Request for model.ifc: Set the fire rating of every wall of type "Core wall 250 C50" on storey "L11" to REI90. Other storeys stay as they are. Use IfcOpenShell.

First a look at what the model holds.

```python
import ifcopenshell
import ifcopenshell.util.element

model = ifcopenshell.open("model.ifc")
print(model.schema)
storey = next(s for s in model.by_type("IfcBuildingStorey") if s.Name == "L11")
walls = [e for e in ifcopenshell.util.element.get_decomposition(storey) if e.is_a("IfcWall")]
seen = {}
for e in walls:
    element_type = ifcopenshell.util.element.get_type(e)
    key = (element_type.Name if element_type != e and element_type else None, ifcopenshell.util.element.get_pset(e, "Pset_WallCommon", "FireRating"))
    seen[key] = seen.get(key, 0) + 1
for (name, value), count in sorted(seen.items(), key=str):
    print(count, "x", name, "|", value)
```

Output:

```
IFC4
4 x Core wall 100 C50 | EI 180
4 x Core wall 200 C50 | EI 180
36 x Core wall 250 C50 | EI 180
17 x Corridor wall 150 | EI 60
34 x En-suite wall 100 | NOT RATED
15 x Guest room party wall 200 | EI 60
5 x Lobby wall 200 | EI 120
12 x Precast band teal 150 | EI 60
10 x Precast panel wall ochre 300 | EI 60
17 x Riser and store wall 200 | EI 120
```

```python
import ifcopenshell
import ifcopenshell.api.pset
import ifcopenshell.util.element

model = ifcopenshell.open("model.ifc")

storey = next(s for s in model.by_type("IfcBuildingStorey") if s.Name == "L11")
walls = [e for e in ifcopenshell.util.element.get_decomposition(storey) if e.is_a("IfcWall")]

count = 0
for e in walls:
    element_type = ifcopenshell.util.element.get_type(e)
    if element_type in (None, e) or element_type.Name != "Core wall 250 C50":
        continue
    # add_pset returns the element's existing set when there is one.
    pset = ifcopenshell.api.pset.add_pset(model, product=e, name="Pset_WallCommon")
    ifcopenshell.api.pset.edit_pset(model, pset=pset, properties={"FireRating": "REI90"})
    count += 1

print(count, "walls updated")

model.write("model_edited.ifc")
```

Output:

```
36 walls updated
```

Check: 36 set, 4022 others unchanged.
